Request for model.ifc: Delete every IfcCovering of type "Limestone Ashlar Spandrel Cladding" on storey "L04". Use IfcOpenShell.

First a look at what the model holds.

```python
import ifcopenshell
import ifcopenshell.util.element

model = ifcopenshell.open("model.ifc")
print(model.schema)
storey = next(s for s in model.by_type("IfcBuildingStorey") if s.Name == "L04")
coverings = [e for e in ifcopenshell.util.element.get_decomposition(storey) if e.is_a("IfcCovering")]
seen = {}
for e in coverings:
    element_type = ifcopenshell.util.element.get_type(e)
    name = element_type.Name if element_type not in (None, e) else None
    seen[name] = seen.get(name, 0) + 1
for name, count in sorted(seen.items(), key=str):
    print(count, "x", name)
```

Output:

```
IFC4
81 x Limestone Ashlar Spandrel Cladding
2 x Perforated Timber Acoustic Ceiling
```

```python
import ifcopenshell
import ifcopenshell.api.root
import ifcopenshell.util.element

model = ifcopenshell.open("model.ifc")

storey = next(s for s in model.by_type("IfcBuildingStorey") if s.Name == "L04")
coverings = [e for e in ifcopenshell.util.element.get_decomposition(storey) if e.is_a("IfcCovering")]
targets = [e for e in coverings if (t := ifcopenshell.util.element.get_type(e)) not in (None, e) and t.Name == "Limestone Ashlar Spandrel Cladding"]

for e in targets:
    ifcopenshell.api.root.remove_product(model, product=e)
print(len(targets), "removed")

model.write("model_v2.ifc")
```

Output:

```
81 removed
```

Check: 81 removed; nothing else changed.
